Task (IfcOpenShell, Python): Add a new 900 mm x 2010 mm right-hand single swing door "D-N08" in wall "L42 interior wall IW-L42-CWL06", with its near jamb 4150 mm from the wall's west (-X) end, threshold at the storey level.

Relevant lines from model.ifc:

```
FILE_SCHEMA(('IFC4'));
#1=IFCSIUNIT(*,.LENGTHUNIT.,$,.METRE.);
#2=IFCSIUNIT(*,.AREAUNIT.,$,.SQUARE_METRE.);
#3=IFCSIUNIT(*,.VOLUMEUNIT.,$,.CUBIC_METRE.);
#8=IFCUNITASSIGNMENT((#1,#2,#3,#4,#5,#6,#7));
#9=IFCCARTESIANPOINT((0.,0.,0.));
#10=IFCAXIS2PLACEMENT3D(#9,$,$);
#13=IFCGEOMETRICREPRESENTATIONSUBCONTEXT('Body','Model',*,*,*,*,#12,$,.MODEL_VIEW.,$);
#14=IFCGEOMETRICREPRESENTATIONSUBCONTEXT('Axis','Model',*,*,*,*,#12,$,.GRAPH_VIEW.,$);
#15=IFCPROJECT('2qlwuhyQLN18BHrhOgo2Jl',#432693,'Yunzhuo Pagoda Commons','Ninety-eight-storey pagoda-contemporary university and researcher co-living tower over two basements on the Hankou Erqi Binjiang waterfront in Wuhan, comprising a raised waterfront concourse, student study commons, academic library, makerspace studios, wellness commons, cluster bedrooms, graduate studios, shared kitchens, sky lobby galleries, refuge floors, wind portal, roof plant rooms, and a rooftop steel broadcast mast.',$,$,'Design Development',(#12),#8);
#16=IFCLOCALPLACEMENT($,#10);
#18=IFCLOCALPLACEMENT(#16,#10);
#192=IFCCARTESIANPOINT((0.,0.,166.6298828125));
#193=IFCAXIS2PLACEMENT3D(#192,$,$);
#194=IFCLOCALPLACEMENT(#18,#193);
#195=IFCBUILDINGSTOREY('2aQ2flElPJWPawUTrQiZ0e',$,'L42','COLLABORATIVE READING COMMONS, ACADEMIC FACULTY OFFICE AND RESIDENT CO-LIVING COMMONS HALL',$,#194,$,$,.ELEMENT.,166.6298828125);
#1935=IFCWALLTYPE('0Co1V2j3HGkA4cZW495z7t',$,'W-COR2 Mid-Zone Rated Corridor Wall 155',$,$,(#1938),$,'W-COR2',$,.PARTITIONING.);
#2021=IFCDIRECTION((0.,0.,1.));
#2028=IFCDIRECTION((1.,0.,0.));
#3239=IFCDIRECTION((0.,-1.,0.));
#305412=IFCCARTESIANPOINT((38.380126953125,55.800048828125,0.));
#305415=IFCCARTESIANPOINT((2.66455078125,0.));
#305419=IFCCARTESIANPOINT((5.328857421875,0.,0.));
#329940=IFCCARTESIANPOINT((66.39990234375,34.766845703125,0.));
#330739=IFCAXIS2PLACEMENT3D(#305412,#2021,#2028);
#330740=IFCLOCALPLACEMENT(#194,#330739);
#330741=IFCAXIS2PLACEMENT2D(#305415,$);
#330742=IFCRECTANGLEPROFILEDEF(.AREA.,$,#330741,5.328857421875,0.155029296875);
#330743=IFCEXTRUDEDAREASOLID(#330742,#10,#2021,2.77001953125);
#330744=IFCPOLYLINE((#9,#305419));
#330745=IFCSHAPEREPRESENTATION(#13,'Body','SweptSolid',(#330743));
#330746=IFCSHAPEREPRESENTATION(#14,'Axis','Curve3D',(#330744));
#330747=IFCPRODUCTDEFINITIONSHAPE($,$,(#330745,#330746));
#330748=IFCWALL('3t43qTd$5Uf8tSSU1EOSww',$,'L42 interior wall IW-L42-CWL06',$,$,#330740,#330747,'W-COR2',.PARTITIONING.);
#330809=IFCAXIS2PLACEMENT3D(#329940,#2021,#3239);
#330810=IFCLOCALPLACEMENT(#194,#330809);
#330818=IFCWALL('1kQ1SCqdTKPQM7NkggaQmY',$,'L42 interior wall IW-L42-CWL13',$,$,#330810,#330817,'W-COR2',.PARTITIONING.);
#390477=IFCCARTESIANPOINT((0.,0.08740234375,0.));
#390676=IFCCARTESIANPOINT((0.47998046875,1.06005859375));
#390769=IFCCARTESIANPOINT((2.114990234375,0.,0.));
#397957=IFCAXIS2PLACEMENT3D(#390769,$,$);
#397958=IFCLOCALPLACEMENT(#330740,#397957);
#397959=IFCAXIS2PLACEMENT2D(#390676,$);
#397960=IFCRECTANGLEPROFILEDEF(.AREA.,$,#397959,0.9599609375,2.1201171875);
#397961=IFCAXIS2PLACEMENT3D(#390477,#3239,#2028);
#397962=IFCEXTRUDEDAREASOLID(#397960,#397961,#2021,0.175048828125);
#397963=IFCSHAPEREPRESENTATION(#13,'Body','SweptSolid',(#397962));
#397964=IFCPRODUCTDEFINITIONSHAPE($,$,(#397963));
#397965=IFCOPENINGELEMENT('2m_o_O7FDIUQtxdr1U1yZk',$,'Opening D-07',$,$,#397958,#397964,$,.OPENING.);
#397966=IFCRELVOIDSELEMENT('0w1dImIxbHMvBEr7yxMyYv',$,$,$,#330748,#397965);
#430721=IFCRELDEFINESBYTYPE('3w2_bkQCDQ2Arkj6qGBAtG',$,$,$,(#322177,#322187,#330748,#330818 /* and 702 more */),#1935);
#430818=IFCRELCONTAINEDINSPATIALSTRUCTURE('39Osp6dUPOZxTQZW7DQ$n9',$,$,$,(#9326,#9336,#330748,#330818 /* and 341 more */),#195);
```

```python
import numpy as np
import ifcopenshell
import ifcopenshell.api.feature
import ifcopenshell.api.geometry
import ifcopenshell.api.root
import ifcopenshell.api.spatial
import ifcopenshell.geom
import ifcopenshell.util.element
import ifcopenshell.util.placement
import ifcopenshell.util.representation
import ifcopenshell.util.shape
import ifcopenshell.util.unit

model = ifcopenshell.open("model.ifc")
unit_scale = ifcopenshell.util.unit.calculate_unit_scale(model)
settings = ifcopenshell.geom.settings()


def volume(element):
    """Net volume in cubic metres, openings subtracted."""
    shape = ifcopenshell.geom.create_shape(settings, element)
    return ifcopenshell.util.shape.get_volume(shape.geometry)


wall = model.by_guid("3t43qTd$5Uf8tSSU1EOSww")
storey = ifcopenshell.util.element.get_container(wall, ifc_class="IfcBuildingStorey")
context = ifcopenshell.util.representation.get_context(model, "Model", "Body", "MODEL_VIEW")
before = volume(wall)

width, height, from_end, sill = 0.9, 2.01, 4.15, 0.0  # metres

# The wall runs along its own X axis, and the end named is its -X end.
wall_shape = ifcopenshell.geom.create_shape(settings, wall)
x, y, z = ifcopenshell.util.shape.get_vertices(wall_shape.geometry).T
start = x.min() + from_end
face, thickness = float(y.min()), float(y.max() - y.min())
wall_matrix = ifcopenshell.util.placement.get_local_placement(wall.ObjectPlacement)
level = ifcopenshell.util.placement.get_local_placement(storey.ObjectPlacement)[2, 3]


def in_wall(x, y):
    """Placement at x, y metres in the wall's axes, at sill height."""
    matrix = wall_matrix.copy()
    matrix[:, 3] = wall_matrix @ np.array([x / unit_scale, y / unit_scale, 0.0, 1.0])
    matrix[2, 3] = level + sill / unit_scale
    return matrix


# Opening: a box that overshoots both wall faces by 50 mm.
opening = ifcopenshell.api.root.create_entity(model, ifc_class="IfcOpeningElement", predefined_type="OPENING")
box = ifcopenshell.api.geometry.add_wall_representation(
    model, context=context, length=width, height=height, thickness=thickness + 0.1
)
ifcopenshell.api.geometry.assign_representation(model, product=opening, representation=box)
ifcopenshell.api.geometry.edit_object_placement(model, product=opening, matrix=in_wall(start, face - 0.05), is_si=False)
ifcopenshell.api.feature.add_feature(model, feature=opening, element=wall)

door = ifcopenshell.api.root.create_entity(model, ifc_class="IfcDoor", name="D-N08", predefined_type="DOOR")
door.OverallWidth, door.OverallHeight = width / unit_scale, height / unit_scale
door.OperationType = "SINGLE_SWING_RIGHT"
body = ifcopenshell.api.geometry.add_door_representation(
    model,
    context=context,
    overall_width=door.OverallWidth,
    overall_height=door.OverallHeight,
    operation_type="SINGLE_SWING_RIGHT",
    lining_properties={"LiningDepth": thickness / unit_scale, "ThresholdDepth": thickness / unit_scale},
)
ifcopenshell.api.geometry.assign_representation(model, product=door, representation=body)
ifcopenshell.api.spatial.assign_container(model, products=[door], relating_structure=storey)
ifcopenshell.api.feature.add_filling(model, opening=opening, element=door)

# The lining spans the wall, so the door starts at the wall face.
ifcopenshell.api.geometry.edit_object_placement(model, product=door, matrix=in_wall(start, face), is_si=False)

after = volume(wall)

print(f"wall volume {before:.3f} -> {after:.3f} m3")

model.write("model-out.ifc")
```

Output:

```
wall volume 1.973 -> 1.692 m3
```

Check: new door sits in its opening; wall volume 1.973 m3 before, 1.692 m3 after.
